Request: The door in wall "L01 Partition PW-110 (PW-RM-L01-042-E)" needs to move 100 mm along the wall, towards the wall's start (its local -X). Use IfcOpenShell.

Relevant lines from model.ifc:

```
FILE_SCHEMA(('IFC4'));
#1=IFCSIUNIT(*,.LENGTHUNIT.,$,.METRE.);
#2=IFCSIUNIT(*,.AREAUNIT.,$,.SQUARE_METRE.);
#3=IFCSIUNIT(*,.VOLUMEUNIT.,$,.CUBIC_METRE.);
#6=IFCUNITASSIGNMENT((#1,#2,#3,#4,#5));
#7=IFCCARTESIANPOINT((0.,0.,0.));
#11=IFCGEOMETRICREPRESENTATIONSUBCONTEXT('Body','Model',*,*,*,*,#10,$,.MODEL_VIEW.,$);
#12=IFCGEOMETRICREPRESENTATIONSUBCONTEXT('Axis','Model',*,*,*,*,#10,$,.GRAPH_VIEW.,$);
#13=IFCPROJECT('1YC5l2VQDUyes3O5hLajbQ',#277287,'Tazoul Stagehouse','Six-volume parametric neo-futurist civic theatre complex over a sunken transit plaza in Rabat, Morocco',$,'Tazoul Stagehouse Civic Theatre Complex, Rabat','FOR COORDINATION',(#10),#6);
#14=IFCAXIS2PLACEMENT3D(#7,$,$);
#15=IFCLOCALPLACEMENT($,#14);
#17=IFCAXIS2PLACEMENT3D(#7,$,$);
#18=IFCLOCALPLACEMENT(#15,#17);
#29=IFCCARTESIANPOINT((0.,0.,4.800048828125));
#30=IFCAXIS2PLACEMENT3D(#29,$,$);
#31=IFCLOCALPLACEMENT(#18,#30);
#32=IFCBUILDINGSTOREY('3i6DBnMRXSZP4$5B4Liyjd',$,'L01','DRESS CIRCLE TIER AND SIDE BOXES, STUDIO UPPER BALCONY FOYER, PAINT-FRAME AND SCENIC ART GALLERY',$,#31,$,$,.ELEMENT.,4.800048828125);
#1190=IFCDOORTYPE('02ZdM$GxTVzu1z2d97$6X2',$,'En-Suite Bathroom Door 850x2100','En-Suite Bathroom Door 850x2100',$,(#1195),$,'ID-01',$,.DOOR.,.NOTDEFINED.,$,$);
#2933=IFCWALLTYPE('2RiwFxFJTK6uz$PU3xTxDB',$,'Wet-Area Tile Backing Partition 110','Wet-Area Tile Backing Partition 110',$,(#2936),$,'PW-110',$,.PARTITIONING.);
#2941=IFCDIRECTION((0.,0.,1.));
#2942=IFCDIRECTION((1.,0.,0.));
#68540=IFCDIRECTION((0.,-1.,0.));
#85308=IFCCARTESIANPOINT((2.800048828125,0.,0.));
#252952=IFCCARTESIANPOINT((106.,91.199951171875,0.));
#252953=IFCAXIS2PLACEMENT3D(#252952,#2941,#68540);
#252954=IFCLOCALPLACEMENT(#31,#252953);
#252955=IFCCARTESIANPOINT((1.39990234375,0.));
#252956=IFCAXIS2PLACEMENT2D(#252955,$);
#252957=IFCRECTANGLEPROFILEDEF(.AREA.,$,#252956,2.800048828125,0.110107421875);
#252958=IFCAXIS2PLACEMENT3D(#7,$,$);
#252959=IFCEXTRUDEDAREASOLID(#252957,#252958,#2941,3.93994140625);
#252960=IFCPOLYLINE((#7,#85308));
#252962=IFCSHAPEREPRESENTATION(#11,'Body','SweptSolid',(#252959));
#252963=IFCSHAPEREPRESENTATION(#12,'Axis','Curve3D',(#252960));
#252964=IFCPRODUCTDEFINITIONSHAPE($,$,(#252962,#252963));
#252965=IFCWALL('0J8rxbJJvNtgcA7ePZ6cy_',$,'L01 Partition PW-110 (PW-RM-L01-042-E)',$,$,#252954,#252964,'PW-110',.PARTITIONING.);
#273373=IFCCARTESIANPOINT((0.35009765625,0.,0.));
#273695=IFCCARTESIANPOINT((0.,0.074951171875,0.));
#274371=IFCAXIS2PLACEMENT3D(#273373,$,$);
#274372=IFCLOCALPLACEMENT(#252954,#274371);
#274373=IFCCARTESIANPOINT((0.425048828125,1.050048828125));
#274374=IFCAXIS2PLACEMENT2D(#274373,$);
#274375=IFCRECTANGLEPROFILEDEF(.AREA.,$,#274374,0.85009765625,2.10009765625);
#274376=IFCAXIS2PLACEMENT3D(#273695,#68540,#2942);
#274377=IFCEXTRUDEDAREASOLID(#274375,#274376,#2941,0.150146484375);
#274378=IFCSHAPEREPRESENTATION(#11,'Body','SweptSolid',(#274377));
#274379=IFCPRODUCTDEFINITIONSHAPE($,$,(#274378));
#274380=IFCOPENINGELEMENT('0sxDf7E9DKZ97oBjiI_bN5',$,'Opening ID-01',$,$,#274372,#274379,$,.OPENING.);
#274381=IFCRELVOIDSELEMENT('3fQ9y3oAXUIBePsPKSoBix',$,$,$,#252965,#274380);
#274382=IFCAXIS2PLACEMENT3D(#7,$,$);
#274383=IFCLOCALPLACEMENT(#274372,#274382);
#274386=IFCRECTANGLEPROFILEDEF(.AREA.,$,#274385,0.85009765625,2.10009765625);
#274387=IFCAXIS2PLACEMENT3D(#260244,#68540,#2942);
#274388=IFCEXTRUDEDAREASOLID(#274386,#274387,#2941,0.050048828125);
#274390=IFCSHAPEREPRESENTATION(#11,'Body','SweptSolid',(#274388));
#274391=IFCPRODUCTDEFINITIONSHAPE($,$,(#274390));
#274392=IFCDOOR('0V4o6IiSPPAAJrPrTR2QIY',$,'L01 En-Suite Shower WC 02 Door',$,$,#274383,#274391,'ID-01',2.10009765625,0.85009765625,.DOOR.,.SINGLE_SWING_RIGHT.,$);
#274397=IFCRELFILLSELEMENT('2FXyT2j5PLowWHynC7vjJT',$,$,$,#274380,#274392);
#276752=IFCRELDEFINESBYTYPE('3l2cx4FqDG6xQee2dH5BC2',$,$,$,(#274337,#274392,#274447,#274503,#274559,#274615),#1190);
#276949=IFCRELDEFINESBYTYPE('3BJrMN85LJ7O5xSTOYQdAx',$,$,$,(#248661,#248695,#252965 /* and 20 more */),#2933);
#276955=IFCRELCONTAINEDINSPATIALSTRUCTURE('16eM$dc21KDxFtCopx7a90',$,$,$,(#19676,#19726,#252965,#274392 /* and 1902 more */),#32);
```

```python
import ifcopenshell
import ifcopenshell.api.geometry
import ifcopenshell.util.placement
import ifcopenshell.util.unit

model = ifcopenshell.open("model.ifc")
unit_scale = ifcopenshell.util.unit.calculate_unit_scale(model)

door = model.by_guid("0V4o6IiSPPAAJrPrTR2QIY")
opening = door.FillsVoids[0].RelatingOpeningElement
wall = opening.VoidsElements[0].RelatingBuildingElement

wall_matrix = ifcopenshell.util.placement.get_local_placement(wall.ObjectPlacement)
shift = wall_matrix[:3, 0] * -0.1 / unit_scale
before = ifcopenshell.util.placement.get_local_placement(door.ObjectPlacement)[:3, 3].copy()

# The door is placed relative to its opening, so it follows when the opening moves.
matrix = ifcopenshell.util.placement.get_local_placement(opening.ObjectPlacement)
matrix[:3, 3] += shift
ifcopenshell.api.geometry.edit_object_placement(
    model, product=opening, matrix=matrix, is_si=False, should_transform_children=True
)

after = ifcopenshell.util.placement.get_local_placement(door.ObjectPlacement)[:3, 3]
print("door moved by", (after - before).round(3) + 0.0)

model.write("model-out.ifc")
```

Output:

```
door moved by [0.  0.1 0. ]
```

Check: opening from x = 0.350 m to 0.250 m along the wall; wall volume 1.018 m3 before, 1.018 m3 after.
